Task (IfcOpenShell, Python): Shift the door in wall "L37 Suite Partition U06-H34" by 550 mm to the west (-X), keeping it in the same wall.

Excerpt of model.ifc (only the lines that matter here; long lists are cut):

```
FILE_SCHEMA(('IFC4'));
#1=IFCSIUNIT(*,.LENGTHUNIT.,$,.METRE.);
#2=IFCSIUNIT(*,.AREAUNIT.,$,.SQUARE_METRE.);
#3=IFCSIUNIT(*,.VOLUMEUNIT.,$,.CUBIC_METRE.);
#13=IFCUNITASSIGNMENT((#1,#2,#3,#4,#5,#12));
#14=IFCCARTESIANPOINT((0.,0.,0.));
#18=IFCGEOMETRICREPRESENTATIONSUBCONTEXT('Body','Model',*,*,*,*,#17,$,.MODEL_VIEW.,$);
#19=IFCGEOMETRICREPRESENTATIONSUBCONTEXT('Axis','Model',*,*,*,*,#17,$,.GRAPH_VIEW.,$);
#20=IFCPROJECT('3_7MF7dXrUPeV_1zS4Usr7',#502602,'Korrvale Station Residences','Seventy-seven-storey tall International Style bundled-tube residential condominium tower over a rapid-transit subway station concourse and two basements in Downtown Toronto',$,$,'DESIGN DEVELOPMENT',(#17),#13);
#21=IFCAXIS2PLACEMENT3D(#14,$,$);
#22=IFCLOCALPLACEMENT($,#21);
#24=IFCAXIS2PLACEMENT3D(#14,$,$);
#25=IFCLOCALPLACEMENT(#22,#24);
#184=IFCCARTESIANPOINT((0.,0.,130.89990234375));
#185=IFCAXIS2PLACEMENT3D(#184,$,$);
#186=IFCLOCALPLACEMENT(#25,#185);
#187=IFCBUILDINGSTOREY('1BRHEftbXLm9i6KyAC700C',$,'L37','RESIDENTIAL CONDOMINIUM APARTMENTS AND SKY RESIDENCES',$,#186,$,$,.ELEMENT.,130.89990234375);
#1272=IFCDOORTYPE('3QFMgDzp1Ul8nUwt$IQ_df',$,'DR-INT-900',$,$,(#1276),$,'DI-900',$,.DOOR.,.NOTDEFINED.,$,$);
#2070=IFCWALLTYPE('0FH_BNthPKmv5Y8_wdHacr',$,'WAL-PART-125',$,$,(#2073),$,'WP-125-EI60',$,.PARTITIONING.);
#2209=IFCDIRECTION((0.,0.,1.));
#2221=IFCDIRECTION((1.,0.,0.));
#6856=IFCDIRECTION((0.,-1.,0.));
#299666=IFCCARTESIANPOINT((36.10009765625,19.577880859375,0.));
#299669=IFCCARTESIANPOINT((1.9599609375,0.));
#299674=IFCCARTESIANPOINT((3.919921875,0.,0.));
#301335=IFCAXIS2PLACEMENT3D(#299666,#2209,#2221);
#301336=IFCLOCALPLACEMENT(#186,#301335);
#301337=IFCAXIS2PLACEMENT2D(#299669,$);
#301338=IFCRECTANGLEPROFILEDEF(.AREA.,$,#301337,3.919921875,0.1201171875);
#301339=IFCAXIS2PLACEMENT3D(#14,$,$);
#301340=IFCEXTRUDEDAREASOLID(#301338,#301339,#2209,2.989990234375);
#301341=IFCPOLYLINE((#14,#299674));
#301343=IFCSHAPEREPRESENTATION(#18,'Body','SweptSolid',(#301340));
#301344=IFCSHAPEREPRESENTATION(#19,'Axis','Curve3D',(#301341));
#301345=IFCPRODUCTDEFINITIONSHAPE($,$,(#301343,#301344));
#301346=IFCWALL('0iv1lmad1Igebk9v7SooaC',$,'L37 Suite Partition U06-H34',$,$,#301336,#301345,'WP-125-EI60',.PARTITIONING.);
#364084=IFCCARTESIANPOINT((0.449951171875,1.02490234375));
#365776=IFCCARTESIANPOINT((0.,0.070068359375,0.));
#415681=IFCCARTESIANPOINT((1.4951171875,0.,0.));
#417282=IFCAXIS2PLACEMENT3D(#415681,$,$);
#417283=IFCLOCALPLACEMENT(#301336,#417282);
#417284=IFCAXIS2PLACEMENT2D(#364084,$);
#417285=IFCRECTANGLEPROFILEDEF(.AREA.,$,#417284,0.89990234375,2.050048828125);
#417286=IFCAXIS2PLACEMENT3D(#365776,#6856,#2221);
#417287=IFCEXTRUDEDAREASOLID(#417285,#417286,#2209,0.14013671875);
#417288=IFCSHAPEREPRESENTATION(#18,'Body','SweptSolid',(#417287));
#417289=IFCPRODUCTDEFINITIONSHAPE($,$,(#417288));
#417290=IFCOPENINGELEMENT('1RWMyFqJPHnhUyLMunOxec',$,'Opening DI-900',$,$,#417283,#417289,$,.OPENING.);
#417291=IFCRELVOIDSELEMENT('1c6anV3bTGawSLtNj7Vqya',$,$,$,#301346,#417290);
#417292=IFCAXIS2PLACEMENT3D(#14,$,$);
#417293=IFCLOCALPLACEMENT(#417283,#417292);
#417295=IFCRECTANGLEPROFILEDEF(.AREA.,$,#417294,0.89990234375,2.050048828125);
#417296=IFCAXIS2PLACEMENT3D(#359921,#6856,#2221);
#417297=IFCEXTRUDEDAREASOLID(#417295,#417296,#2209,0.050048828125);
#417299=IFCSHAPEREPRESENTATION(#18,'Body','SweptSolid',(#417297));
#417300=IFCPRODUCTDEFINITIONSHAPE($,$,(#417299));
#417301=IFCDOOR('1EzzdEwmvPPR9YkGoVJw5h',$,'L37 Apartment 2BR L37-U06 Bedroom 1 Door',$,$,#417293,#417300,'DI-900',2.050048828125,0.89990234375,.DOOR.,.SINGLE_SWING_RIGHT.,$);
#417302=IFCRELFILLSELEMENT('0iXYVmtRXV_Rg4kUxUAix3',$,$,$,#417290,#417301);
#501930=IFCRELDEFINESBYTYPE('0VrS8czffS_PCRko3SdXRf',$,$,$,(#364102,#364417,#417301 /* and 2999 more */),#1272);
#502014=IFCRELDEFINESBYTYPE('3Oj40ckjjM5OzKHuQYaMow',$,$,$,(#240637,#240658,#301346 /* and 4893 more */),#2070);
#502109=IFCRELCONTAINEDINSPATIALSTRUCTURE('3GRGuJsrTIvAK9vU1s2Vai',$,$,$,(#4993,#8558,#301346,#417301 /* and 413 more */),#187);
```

```python
import ifcopenshell
import ifcopenshell.api.geometry
import ifcopenshell.util.placement

model = ifcopenshell.open("model.ifc")

door = model.by_id(417301)
opening = door.FillsVoids[0].RelatingOpeningElement
wall = opening.VoidsElements[0].RelatingBuildingElement

wall_matrix = ifcopenshell.util.placement.get_local_placement(wall.ObjectPlacement)
shift = wall_matrix[:3, 0] * -0.55
before = ifcopenshell.util.placement.get_local_placement(door.ObjectPlacement)[:3, 3].copy()

# The door is placed relative to its opening, so it follows when the opening moves.
matrix = ifcopenshell.util.placement.get_local_placement(opening.ObjectPlacement)
matrix[:3, 3] += shift
ifcopenshell.api.geometry.edit_object_placement(
    model, product=opening, matrix=matrix, is_si=False, should_transform_children=True
)

after = ifcopenshell.util.placement.get_local_placement(door.ObjectPlacement)[:3, 3]
print("door moved by", (after - before).round(3) + 0.0)

model.write("model_v2.ifc")
```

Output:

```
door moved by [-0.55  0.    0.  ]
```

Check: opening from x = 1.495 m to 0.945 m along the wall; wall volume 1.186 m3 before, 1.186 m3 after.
